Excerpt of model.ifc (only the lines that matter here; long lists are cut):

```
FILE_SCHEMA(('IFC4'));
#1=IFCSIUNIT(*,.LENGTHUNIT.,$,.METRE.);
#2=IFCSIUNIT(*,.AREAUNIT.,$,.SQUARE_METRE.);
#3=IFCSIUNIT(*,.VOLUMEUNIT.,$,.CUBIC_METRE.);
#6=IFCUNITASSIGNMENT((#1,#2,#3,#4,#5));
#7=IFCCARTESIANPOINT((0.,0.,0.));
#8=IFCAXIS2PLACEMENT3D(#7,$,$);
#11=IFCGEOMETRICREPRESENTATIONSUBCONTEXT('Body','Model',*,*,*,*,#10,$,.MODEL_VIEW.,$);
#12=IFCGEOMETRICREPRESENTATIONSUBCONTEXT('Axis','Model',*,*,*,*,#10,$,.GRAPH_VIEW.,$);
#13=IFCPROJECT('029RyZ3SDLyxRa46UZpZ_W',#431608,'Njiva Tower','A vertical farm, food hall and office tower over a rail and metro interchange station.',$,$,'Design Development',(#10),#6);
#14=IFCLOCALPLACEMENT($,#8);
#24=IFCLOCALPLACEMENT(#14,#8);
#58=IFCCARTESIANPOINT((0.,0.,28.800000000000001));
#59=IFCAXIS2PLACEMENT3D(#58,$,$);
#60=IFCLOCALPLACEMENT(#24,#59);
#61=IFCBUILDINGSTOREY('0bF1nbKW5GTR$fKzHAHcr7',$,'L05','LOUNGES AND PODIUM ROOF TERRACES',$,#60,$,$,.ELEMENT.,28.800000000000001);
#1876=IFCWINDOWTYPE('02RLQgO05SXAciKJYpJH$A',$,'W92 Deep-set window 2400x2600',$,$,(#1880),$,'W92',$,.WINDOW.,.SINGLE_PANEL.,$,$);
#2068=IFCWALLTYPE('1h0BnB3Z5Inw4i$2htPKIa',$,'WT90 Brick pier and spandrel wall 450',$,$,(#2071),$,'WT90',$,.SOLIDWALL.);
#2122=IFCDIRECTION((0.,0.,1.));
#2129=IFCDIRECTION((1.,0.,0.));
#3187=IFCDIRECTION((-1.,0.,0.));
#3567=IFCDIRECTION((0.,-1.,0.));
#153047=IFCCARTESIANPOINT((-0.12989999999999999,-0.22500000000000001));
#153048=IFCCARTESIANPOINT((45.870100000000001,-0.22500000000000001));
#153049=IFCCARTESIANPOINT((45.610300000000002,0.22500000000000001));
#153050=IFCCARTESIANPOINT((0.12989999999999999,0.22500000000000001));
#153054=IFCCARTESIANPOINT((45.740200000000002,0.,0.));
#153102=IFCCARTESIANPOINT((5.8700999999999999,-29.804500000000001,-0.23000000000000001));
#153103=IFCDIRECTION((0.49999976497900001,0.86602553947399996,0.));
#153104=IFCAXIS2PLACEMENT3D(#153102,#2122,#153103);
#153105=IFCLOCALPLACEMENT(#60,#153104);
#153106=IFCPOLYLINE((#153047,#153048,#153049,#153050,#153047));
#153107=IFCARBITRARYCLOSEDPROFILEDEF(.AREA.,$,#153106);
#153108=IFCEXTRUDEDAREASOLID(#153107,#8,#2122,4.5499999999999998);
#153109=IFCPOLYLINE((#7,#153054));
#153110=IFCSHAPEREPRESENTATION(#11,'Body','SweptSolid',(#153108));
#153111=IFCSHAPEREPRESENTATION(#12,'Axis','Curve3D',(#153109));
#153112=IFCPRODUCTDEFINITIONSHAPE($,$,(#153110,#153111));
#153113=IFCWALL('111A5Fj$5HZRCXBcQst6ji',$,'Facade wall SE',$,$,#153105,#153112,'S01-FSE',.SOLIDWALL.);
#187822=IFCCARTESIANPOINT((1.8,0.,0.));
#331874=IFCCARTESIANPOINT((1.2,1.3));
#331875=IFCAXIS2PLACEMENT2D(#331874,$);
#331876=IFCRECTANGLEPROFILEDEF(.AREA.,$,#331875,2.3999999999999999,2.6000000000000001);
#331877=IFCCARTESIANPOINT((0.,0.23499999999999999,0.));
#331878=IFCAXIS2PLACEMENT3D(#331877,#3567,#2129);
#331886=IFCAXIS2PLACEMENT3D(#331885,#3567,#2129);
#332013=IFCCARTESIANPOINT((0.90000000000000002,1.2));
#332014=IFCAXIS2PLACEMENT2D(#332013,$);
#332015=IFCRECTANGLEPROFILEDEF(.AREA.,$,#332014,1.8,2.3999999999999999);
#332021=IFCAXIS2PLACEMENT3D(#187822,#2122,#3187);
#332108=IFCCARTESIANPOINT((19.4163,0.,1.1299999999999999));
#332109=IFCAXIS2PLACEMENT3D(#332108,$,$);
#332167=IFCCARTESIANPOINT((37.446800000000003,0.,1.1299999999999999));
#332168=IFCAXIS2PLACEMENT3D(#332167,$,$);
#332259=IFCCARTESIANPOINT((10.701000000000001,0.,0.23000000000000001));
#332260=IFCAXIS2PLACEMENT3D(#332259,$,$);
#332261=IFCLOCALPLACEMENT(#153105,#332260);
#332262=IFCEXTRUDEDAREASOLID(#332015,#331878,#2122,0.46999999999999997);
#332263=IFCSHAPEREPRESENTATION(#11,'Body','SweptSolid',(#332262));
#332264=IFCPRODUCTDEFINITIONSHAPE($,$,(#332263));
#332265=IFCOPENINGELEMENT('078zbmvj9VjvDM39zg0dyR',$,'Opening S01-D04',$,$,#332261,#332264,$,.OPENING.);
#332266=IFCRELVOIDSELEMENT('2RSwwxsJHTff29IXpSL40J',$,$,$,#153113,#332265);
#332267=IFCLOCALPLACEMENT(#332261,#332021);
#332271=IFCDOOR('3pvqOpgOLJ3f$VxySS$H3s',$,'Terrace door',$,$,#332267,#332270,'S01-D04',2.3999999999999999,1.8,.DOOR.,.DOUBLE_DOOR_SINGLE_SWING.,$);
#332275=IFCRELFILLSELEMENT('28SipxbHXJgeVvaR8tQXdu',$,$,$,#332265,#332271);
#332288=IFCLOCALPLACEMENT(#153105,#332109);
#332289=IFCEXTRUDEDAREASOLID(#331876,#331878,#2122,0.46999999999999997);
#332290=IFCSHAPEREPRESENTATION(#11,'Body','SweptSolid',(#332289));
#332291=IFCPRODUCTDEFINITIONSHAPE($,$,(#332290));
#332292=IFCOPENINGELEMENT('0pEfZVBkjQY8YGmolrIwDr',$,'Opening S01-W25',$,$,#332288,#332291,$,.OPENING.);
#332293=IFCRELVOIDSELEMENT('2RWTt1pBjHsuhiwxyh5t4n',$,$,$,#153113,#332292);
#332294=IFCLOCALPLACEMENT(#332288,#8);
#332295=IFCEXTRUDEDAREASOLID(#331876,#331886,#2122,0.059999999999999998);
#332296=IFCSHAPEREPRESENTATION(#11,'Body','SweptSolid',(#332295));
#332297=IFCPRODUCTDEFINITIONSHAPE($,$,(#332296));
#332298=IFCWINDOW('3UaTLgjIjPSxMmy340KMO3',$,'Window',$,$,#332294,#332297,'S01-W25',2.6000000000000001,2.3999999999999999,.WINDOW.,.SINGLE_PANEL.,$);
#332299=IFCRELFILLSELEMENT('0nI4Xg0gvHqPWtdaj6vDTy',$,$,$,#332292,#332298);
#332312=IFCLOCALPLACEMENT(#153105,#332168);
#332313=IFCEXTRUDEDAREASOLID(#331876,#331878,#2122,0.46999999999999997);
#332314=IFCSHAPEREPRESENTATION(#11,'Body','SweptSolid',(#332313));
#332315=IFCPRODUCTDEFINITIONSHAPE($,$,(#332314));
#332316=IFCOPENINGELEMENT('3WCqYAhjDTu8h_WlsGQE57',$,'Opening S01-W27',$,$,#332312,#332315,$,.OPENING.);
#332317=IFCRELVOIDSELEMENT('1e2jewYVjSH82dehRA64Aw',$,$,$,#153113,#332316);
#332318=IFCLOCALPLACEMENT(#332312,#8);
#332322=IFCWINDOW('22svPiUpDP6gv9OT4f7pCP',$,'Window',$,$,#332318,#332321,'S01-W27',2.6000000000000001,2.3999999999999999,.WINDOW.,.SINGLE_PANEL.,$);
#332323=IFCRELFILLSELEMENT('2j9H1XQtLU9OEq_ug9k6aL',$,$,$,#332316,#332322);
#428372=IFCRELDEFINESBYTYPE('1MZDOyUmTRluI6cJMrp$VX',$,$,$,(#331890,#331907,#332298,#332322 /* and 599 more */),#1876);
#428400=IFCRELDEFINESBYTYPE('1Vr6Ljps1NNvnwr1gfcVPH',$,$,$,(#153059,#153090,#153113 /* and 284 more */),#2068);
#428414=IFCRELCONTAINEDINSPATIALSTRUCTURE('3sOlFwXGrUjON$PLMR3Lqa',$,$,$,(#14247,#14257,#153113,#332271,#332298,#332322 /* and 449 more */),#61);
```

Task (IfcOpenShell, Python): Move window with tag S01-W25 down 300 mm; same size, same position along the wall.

```python
import numpy as np
import ifcopenshell
import ifcopenshell.api.geometry
import ifcopenshell.util.placement
import ifcopenshell.util.unit

model = ifcopenshell.open("model.ifc")
unit_scale = ifcopenshell.util.unit.calculate_unit_scale(model)

window = model.by_id(332298)
opening = window.FillsVoids[0].RelatingOpeningElement
dz = -0.3 / unit_scale

shift = np.array([0.0, 0.0, dz])
# The window is placed relative to its opening, so it follows when the opening moves.
matrix = ifcopenshell.util.placement.get_local_placement(opening.ObjectPlacement)
matrix[:3, 3] += shift
ifcopenshell.api.geometry.edit_object_placement(
    model, product=opening, matrix=matrix, is_si=False, should_transform_children=True
)

print(f"moved by {dz * unit_scale:+.3f} m")

model.write("model_edited.ifc")
```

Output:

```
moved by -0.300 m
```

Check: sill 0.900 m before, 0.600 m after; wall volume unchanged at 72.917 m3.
